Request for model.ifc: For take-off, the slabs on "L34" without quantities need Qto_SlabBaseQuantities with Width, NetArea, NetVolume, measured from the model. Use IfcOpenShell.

First a look at what the model holds.

```python
import ifcopenshell
import ifcopenshell.util.element
import ifcopenshell.util.unit

model = ifcopenshell.open("model.ifc")
print(model.schema)
for unit_type in ("LENGTHUNIT", "AREAUNIT", "VOLUMEUNIT"):
    print(unit_type, ifcopenshell.util.unit.calculate_unit_scale(model, unit_type))
storey = next(s for s in model.by_type("IfcBuildingStorey") if s.Name == "L34")
slabs = [e for e in ifcopenshell.util.element.get_decomposition(storey) if e.is_a("IfcSlab")]
for e in sorted(slabs, key=lambda e: e.id()):
    print(e.id(), e.is_a(), e.Name, list(ifcopenshell.util.element.get_psets(e, qtos_only=True)), sep=" | ")
```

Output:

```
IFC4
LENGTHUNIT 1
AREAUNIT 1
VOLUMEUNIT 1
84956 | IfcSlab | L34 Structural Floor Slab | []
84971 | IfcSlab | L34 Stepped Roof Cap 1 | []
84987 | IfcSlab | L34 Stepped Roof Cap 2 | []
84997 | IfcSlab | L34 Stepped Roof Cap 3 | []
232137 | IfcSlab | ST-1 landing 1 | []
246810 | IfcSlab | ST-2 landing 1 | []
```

```python
import ifcopenshell
import ifcopenshell.api.pset
import ifcopenshell.geom
import ifcopenshell.util.element
import ifcopenshell.util.shape
import ifcopenshell.util.unit

model = ifcopenshell.open("model.ifc")
unit_scale = ifcopenshell.util.unit.calculate_unit_scale(model)
area_scale = ifcopenshell.util.unit.calculate_unit_scale(model, "AREAUNIT")
volume_scale = ifcopenshell.util.unit.calculate_unit_scale(model, "VOLUMEUNIT")
settings = ifcopenshell.geom.settings()

storey = next(s for s in model.by_type("IfcBuildingStorey") if s.Name == "L34")
slabs = [e for e in ifcopenshell.util.element.get_decomposition(storey) if e.is_a("IfcSlab")]

for e in sorted(slabs, key=lambda e: e.id()):
    if ifcopenshell.util.element.get_psets(e, qtos_only=True, should_inherit=False):
        continue
    # Geometry comes back in metres, in the element's own axes.
    shape = ifcopenshell.geom.create_shape(settings, e)
    values = {
        "Width": ifcopenshell.util.shape.get_z(shape.geometry) / unit_scale,
        "NetArea": ifcopenshell.util.shape.get_footprint_area(shape.geometry) / area_scale,
        "NetVolume": ifcopenshell.util.shape.get_volume(shape.geometry) / volume_scale,
    }
    qto = ifcopenshell.api.pset.add_qto(model, product=e, name="Qto_SlabBaseQuantities")
    ifcopenshell.api.pset.edit_qto(model, qto=qto, properties=values)
    print(e.id(), {k: round(v, 3) for k, v in values.items()})

model.write("model_rev.ifc")
```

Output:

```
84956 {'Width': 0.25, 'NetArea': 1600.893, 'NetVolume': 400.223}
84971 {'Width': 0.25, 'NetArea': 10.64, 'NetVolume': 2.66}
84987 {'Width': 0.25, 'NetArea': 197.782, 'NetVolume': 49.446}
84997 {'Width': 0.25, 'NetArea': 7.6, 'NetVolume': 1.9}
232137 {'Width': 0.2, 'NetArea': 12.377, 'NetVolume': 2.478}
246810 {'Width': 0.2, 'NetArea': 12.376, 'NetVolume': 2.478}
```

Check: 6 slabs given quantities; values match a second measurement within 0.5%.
